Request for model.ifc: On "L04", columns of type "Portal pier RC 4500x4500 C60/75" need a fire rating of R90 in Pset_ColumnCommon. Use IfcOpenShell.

First a look at what the model holds.

```python
import ifcopenshell
import ifcopenshell.util.element

model = ifcopenshell.open("model.ifc")
print(model.schema)
storey = next(s for s in model.by_type("IfcBuildingStorey") if s.Name == "L04")
columns = [e for e in ifcopenshell.util.element.get_decomposition(storey) if e.is_a("IfcColumn")]
seen = {}
for e in columns:
    element_type = ifcopenshell.util.element.get_type(e)
    key = (element_type.Name if element_type != e and element_type else None, ifcopenshell.util.element.get_pset(e, "Pset_ColumnCommon", "FireRating"))
    seen[key] = seen.get(key, 0) + 1
for (name, value), count in sorted(seen.items(), key=str):
    print(count, "x", name, "|", value)
```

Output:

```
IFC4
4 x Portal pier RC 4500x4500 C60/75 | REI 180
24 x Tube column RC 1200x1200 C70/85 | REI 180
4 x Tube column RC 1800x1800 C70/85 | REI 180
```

```python
import ifcopenshell
import ifcopenshell.api.pset
import ifcopenshell.util.element

model = ifcopenshell.open("model.ifc")

storey = next(s for s in model.by_type("IfcBuildingStorey") if s.Name == "L04")
columns = [e for e in ifcopenshell.util.element.get_decomposition(storey) if e.is_a("IfcColumn")]

count = 0
for e in columns:
    element_type = ifcopenshell.util.element.get_type(e)
    if element_type in (None, e) or element_type.Name != "Portal pier RC 4500x4500 C60/75":
        continue
    found = ifcopenshell.util.element.get_pset(e, "Pset_ColumnCommon", should_inherit=False)
    if found:
        pset = model.by_id(found["id"])
        if len(ifcopenshell.util.element.get_elements_by_pset(pset)) > 1:
            pset = ifcopenshell.api.pset.unshare_pset(model, products=[e], pset=pset)[0]
    else:
        pset = ifcopenshell.api.pset.add_pset(model, product=e, name="Pset_ColumnCommon")
    ifcopenshell.api.pset.edit_pset(model, pset=pset, properties={"FireRating": "R90"})
    count += 1

print(count, "columns updated")

model.write("model_v2.ifc")
```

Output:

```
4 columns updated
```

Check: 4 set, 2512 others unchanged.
